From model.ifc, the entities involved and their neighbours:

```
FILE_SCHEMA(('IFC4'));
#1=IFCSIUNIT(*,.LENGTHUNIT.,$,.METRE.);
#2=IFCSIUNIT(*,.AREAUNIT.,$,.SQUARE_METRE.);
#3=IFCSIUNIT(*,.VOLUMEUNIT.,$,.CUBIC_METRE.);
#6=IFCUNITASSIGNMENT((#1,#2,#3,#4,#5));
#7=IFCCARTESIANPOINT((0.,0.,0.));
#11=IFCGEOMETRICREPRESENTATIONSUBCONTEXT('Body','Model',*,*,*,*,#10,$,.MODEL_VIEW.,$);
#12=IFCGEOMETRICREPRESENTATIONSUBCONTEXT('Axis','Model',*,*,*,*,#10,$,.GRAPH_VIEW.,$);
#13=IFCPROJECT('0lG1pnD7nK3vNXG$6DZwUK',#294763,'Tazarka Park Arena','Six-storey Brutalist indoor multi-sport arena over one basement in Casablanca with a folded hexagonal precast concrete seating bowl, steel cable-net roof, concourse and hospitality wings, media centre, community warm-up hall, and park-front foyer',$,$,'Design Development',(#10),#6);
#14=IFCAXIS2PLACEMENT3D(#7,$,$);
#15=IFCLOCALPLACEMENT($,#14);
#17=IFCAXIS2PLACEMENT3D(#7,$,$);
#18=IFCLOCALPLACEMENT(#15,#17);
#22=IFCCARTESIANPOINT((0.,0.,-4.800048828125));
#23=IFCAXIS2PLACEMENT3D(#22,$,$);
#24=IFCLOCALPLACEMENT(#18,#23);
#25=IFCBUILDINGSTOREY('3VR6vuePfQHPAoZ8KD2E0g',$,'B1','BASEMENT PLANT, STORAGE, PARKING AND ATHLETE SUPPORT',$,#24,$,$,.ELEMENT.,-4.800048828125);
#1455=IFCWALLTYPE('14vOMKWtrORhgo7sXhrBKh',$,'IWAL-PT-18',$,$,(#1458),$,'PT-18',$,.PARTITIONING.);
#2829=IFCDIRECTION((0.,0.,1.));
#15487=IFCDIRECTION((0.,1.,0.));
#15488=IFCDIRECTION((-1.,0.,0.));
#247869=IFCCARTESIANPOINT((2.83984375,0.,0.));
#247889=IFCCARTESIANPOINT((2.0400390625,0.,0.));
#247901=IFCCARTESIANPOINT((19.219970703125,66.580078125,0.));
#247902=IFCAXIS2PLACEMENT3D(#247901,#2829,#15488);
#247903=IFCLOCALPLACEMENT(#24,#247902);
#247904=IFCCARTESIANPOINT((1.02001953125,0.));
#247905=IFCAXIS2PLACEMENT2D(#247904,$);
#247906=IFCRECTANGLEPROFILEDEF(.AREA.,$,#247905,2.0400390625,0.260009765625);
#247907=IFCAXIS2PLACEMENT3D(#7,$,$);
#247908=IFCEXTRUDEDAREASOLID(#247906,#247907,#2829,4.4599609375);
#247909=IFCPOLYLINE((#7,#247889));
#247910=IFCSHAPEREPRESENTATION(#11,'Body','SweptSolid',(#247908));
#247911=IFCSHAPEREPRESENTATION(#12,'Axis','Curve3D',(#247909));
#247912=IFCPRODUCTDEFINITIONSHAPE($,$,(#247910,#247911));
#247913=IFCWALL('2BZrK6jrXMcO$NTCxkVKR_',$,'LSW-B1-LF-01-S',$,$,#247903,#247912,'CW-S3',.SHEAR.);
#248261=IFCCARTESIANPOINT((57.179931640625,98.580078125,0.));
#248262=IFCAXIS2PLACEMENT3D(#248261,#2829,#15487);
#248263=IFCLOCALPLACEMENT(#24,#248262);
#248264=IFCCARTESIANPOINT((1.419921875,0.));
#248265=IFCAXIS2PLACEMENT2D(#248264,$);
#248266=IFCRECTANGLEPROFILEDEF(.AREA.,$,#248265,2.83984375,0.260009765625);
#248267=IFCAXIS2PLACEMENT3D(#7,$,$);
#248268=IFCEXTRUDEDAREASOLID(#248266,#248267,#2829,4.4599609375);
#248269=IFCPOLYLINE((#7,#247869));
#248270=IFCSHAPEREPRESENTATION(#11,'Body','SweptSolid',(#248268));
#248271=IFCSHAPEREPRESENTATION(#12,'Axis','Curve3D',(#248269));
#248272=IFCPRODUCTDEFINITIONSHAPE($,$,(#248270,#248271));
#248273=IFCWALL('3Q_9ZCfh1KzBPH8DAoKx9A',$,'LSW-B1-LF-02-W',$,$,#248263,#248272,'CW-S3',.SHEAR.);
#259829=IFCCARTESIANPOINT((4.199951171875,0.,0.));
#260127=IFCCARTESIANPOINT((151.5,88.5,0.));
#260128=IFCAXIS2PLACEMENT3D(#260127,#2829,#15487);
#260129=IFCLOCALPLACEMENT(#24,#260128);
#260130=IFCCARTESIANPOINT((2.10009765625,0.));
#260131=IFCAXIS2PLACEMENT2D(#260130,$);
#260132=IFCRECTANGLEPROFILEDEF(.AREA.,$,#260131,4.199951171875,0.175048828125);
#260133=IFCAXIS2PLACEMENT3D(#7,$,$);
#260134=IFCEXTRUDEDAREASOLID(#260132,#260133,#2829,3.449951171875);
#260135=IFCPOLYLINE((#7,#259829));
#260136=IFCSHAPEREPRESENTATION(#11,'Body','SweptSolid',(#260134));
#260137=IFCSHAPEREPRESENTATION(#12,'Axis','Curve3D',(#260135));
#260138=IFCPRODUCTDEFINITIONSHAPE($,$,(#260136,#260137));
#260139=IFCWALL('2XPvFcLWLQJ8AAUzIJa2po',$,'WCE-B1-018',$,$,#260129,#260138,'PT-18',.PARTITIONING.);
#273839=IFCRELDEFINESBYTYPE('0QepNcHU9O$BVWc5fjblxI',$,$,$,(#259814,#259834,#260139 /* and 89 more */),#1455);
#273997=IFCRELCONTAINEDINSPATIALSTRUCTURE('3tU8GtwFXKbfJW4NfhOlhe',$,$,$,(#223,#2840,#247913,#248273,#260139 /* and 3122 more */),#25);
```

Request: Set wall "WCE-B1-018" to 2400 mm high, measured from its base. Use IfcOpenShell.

```python
import ifcopenshell
import ifcopenshell.geom
import ifcopenshell.util.representation
import ifcopenshell.util.shape

model = ifcopenshell.open("model.ifc")
settings = ifcopenshell.geom.settings()


def volume(element):
    """Net volume in cubic metres, openings subtracted."""
    shape = ifcopenshell.geom.create_shape(settings, element)
    return ifcopenshell.util.shape.get_volume(shape.geometry)


wall = model.by_guid("2XPvFcLWLQJ8AAUzIJa2po")
before = volume(wall)

body = ifcopenshell.util.representation.get_representation(wall, "Model", "Body")
solid = body.Items[0]
old_height = solid.Depth
solid.Depth = 2.4
after = volume(wall)

print(f"height {old_height:g} -> {solid.Depth:g}, volume {before:.3f} -> {after:.3f} m3")

model.write("model_edited.ifc")
```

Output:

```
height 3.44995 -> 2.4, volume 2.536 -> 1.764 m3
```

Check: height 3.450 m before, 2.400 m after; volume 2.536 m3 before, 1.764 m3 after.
